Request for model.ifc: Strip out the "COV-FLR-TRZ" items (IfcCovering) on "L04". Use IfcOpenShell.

First a look at what the model holds.

```python
import ifcopenshell
import ifcopenshell.util.element

model = ifcopenshell.open("model.ifc")
print(model.schema)
storey = next(s for s in model.by_type("IfcBuildingStorey") if s.Name == "L04")
coverings = [e for e in ifcopenshell.util.element.get_decomposition(storey) if e.is_a("IfcCovering")]
seen = {}
for e in coverings:
    element_type = ifcopenshell.util.element.get_type(e)
    name = element_type.Name if element_type not in (None, e) else None
    seen[name] = seen.get(name, 0) + 1
for name, count in sorted(seen.items(), key=str):
    print(count, "x", name)
```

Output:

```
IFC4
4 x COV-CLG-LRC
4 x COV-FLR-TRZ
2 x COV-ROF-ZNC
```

```python
import ifcopenshell
import ifcopenshell.api.root
import ifcopenshell.util.element

model = ifcopenshell.open("model.ifc")

storey = next(s for s in model.by_type("IfcBuildingStorey") if s.Name == "L04")
coverings = [e for e in ifcopenshell.util.element.get_decomposition(storey) if e.is_a("IfcCovering")]
targets = [e for e in coverings if (t := ifcopenshell.util.element.get_type(e)) not in (None, e) and t.Name == "COV-FLR-TRZ"]

for e in targets:
    ifcopenshell.api.root.remove_product(model, product=e)
print(len(targets), "removed")

model.write("model_rev.ifc")
```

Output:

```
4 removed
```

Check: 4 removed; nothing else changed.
